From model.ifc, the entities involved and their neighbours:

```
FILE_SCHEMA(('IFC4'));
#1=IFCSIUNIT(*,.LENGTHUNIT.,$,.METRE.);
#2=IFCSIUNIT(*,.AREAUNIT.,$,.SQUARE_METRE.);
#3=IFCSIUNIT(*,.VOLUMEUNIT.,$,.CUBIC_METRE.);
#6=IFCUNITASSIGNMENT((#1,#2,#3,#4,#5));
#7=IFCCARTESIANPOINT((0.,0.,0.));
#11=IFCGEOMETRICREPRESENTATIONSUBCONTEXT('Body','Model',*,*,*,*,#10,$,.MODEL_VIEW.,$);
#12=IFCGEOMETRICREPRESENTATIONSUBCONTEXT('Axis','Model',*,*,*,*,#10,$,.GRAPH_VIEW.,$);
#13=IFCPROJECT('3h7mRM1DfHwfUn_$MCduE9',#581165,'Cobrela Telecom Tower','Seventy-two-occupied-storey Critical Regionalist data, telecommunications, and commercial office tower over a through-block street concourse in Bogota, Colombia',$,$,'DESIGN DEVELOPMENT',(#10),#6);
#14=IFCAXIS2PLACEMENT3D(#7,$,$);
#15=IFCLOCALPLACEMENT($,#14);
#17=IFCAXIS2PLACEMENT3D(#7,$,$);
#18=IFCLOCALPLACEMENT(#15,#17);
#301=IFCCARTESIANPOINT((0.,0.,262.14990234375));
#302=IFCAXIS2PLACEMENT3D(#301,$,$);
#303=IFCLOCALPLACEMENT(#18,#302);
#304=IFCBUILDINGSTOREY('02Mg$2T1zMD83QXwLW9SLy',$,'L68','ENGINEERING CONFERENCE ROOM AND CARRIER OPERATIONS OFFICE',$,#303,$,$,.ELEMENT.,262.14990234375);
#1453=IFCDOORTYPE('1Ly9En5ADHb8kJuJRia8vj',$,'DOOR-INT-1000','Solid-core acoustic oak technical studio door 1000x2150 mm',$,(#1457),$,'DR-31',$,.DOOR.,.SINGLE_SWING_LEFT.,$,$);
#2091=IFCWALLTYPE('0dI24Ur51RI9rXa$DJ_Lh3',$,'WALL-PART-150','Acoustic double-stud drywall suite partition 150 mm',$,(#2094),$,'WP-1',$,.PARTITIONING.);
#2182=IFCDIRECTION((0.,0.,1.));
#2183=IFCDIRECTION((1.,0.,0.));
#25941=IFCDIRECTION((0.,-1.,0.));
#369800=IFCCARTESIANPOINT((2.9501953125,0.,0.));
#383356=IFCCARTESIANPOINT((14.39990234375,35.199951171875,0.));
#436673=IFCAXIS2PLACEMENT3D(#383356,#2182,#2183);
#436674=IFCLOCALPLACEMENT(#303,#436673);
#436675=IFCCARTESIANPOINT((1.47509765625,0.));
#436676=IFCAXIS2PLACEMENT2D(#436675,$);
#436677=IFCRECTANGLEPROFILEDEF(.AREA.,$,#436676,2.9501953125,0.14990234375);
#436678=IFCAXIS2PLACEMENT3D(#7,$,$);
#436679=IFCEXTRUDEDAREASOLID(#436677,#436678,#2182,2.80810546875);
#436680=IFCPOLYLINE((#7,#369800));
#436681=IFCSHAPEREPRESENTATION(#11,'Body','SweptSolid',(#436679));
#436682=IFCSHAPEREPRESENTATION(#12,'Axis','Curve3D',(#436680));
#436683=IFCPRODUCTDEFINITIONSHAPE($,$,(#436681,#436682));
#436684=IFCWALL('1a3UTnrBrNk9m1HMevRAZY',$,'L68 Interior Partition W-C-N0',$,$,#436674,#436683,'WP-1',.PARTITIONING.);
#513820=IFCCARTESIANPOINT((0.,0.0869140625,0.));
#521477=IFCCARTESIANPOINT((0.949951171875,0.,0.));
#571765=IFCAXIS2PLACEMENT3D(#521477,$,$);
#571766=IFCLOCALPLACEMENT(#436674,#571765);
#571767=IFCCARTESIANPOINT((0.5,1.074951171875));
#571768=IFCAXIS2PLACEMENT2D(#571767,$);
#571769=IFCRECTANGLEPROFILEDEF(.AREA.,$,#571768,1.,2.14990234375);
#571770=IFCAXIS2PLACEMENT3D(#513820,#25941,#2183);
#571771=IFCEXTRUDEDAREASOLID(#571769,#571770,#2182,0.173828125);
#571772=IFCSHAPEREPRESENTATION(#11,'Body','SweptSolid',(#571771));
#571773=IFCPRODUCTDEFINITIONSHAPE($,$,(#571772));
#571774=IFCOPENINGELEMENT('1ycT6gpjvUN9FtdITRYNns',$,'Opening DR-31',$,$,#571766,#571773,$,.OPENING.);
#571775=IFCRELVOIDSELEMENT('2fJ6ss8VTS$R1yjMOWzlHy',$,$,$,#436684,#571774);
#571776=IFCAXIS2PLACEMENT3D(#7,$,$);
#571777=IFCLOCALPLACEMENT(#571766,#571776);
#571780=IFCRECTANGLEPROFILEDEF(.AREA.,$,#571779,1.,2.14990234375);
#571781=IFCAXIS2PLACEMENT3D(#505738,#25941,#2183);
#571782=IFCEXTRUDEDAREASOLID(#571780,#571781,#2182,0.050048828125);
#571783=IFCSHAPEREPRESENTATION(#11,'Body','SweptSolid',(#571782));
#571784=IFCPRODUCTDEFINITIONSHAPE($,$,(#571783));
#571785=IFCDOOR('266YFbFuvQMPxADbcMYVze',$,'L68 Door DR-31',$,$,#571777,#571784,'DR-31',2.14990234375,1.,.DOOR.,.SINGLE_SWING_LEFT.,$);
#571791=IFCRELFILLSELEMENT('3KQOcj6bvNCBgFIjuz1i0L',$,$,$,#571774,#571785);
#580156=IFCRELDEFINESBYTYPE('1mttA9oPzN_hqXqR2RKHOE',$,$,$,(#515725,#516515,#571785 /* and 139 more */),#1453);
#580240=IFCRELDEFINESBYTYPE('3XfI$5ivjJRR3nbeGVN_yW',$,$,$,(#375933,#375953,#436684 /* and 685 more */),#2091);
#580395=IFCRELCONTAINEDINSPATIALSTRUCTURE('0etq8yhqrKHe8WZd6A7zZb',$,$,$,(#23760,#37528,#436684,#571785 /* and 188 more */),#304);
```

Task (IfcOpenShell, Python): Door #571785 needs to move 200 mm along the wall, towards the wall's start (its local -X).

```python
import ifcopenshell
import ifcopenshell.api.geometry
import ifcopenshell.util.placement

model = ifcopenshell.open("model.ifc")

door = model.by_guid("266YFbFuvQMPxADbcMYVze")
opening = door.FillsVoids[0].RelatingOpeningElement
wall = opening.VoidsElements[0].RelatingBuildingElement

wall_matrix = ifcopenshell.util.placement.get_local_placement(wall.ObjectPlacement)
shift = wall_matrix[:3, 0] * -0.2
before = ifcopenshell.util.placement.get_local_placement(door.ObjectPlacement)[:3, 3].copy()

# The door is placed relative to its opening, so it follows when the opening moves.
matrix = ifcopenshell.util.placement.get_local_placement(opening.ObjectPlacement)
matrix[:3, 3] += shift
ifcopenshell.api.geometry.edit_object_placement(
    model, product=opening, matrix=matrix, is_si=False, should_transform_children=True
)

after = ifcopenshell.util.placement.get_local_placement(door.ObjectPlacement)[:3, 3]
print("door moved by", (after - before).round(3) + 0.0)

model.write("model-out.ifc")
```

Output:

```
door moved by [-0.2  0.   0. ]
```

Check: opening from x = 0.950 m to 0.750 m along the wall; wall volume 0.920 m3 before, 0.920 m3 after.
